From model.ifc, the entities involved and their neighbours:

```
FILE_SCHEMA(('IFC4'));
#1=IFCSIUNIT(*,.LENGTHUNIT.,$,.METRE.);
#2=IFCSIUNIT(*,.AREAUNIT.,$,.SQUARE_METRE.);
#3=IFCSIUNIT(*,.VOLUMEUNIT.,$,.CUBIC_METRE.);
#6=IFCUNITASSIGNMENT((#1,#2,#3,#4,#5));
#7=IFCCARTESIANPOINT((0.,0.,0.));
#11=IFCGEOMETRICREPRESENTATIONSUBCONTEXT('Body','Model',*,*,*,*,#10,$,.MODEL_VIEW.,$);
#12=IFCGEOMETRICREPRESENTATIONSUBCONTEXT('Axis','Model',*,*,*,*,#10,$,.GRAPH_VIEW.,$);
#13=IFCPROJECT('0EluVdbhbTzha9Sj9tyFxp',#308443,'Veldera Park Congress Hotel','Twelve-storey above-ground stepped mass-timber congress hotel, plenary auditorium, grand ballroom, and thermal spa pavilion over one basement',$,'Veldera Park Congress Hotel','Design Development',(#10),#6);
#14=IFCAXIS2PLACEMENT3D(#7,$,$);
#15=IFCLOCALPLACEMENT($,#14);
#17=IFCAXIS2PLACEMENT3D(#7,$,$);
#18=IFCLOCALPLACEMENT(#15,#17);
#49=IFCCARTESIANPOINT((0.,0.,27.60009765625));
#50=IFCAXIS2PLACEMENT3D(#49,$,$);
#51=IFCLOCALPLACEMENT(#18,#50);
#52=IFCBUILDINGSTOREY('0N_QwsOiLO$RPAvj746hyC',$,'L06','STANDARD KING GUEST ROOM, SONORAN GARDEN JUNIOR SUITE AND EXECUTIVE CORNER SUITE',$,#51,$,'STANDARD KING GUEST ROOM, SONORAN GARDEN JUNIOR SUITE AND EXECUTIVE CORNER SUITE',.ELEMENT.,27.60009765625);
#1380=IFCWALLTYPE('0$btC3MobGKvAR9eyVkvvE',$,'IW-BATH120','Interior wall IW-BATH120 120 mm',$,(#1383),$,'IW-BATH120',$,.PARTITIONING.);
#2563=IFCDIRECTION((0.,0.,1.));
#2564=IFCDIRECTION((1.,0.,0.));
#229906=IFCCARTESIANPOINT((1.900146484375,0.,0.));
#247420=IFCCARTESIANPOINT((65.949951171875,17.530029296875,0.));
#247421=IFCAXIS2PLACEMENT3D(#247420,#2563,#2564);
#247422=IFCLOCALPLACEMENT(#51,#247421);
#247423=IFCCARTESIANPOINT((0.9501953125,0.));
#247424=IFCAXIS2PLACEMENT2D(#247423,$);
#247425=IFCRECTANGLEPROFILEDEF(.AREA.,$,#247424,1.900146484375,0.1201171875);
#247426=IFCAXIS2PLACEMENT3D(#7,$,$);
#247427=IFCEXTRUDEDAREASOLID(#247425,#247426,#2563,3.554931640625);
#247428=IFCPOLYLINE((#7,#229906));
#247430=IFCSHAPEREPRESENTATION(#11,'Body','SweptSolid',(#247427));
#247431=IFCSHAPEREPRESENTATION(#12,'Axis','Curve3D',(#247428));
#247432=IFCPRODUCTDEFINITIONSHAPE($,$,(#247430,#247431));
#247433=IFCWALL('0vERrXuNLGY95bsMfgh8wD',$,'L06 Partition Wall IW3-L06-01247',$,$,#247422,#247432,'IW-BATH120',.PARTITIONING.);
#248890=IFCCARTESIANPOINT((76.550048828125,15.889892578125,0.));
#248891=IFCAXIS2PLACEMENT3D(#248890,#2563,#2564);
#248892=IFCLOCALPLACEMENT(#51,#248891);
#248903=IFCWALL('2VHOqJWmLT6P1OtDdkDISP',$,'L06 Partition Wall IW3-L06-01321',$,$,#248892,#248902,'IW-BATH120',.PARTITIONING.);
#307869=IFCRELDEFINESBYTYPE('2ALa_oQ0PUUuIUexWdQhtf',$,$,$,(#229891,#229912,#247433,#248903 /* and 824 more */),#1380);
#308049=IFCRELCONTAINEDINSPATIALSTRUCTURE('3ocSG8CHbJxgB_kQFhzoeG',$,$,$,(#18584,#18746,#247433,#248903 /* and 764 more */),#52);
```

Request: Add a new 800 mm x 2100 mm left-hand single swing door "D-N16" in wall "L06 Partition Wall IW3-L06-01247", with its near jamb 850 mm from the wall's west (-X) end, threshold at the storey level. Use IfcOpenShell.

```python
import numpy as np
import ifcopenshell
import ifcopenshell.api.feature
import ifcopenshell.api.geometry
import ifcopenshell.api.root
import ifcopenshell.api.spatial
import ifcopenshell.geom
import ifcopenshell.util.element
import ifcopenshell.util.placement
import ifcopenshell.util.representation
import ifcopenshell.util.shape
import ifcopenshell.util.unit

model = ifcopenshell.open("model.ifc")
unit_scale = ifcopenshell.util.unit.calculate_unit_scale(model)
settings = ifcopenshell.geom.settings()


def volume(element):
    """Net volume in cubic metres, openings subtracted."""
    shape = ifcopenshell.geom.create_shape(settings, element)
    return ifcopenshell.util.shape.get_volume(shape.geometry)


wall = model.by_guid("0vERrXuNLGY95bsMfgh8wD")
storey = ifcopenshell.util.element.get_container(wall, ifc_class="IfcBuildingStorey")
context = ifcopenshell.util.representation.get_context(model, "Model", "Body", "MODEL_VIEW")
before = volume(wall)

width, height, from_end, sill = 0.8, 2.1, 0.85, 0.0  # metres

# The wall runs along its own X axis, and the end named is its -X end.
wall_shape = ifcopenshell.geom.create_shape(settings, wall)
x, y, z = ifcopenshell.util.shape.get_vertices(wall_shape.geometry).T
start = x.min() + from_end
face, thickness = float(y.min()), float(y.max() - y.min())
wall_matrix = ifcopenshell.util.placement.get_local_placement(wall.ObjectPlacement)
level = ifcopenshell.util.placement.get_local_placement(storey.ObjectPlacement)[2, 3]


def in_wall(x, y):
    """Placement at x, y metres in the wall's axes, at sill height."""
    matrix = wall_matrix.copy()
    matrix[:, 3] = wall_matrix @ np.array([x / unit_scale, y / unit_scale, 0.0, 1.0])
    matrix[2, 3] = level + sill / unit_scale
    return matrix


# Opening: a box that overshoots both wall faces by 50 mm.
opening = ifcopenshell.api.root.create_entity(model, ifc_class="IfcOpeningElement", predefined_type="OPENING")
box = ifcopenshell.api.geometry.add_wall_representation(
    model, context=context, length=width, height=height, thickness=thickness + 0.1
)
ifcopenshell.api.geometry.assign_representation(model, product=opening, representation=box)
ifcopenshell.api.geometry.edit_object_placement(model, product=opening, matrix=in_wall(start, face - 0.05), is_si=False)
ifcopenshell.api.feature.add_feature(model, feature=opening, element=wall)

door = ifcopenshell.api.root.create_entity(model, ifc_class="IfcDoor", name="D-N16", predefined_type="DOOR")
door.OverallWidth, door.OverallHeight = width / unit_scale, height / unit_scale
door.OperationType = "SINGLE_SWING_LEFT"
body = ifcopenshell.api.geometry.add_door_representation(
    model,
    context=context,
    overall_width=door.OverallWidth,
    overall_height=door.OverallHeight,
    operation_type="SINGLE_SWING_LEFT",
    lining_properties={"LiningDepth": thickness / unit_scale, "ThresholdDepth": thickness / unit_scale},
)
ifcopenshell.api.geometry.assign_representation(model, product=door, representation=body)
ifcopenshell.api.spatial.assign_container(model, products=[door], relating_structure=storey)
ifcopenshell.api.feature.add_filling(model, opening=opening, element=door)

# The lining spans the wall, so the door starts at the wall face.
ifcopenshell.api.geometry.edit_object_placement(model, product=door, matrix=in_wall(start, face), is_si=False)

after = volume(wall)

print(f"wall volume {before:.3f} -> {after:.3f} m3")

model.write("model-out.ifc")
```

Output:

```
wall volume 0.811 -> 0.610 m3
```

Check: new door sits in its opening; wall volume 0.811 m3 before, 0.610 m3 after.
